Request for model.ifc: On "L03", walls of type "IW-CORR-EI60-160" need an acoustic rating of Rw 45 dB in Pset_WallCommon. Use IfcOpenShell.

First a look at what the model holds.

```python
import ifcopenshell
import ifcopenshell.util.element

model = ifcopenshell.open("model.ifc")
print(model.schema)
storey = next(s for s in model.by_type("IfcBuildingStorey") if s.Name == "L03")
walls = [e for e in ifcopenshell.util.element.get_decomposition(storey) if e.is_a("IfcWall")]
seen = {}
for e in walls:
    element_type = ifcopenshell.util.element.get_type(e)
    key = (element_type.Name if element_type != e and element_type else None, ifcopenshell.util.element.get_pset(e, "Pset_WallCommon", "AcousticRating"))
    seen[key] = seen.get(key, 0) + 1
for (name, value), count in sorted(seen.items(), key=str):
    print(count, "x", name, "|", value)
```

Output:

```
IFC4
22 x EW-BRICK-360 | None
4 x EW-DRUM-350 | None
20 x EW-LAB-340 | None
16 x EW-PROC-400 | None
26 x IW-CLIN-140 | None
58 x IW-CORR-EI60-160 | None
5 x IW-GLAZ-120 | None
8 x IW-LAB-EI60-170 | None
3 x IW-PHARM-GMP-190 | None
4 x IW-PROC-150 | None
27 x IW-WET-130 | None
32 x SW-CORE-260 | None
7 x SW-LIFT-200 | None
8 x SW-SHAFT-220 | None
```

```python
import ifcopenshell
import ifcopenshell.api.pset
import ifcopenshell.util.element

model = ifcopenshell.open("model.ifc")

storey = next(s for s in model.by_type("IfcBuildingStorey") if s.Name == "L03")
walls = [e for e in ifcopenshell.util.element.get_decomposition(storey) if e.is_a("IfcWall")]

count = 0
for e in walls:
    element_type = ifcopenshell.util.element.get_type(e)
    if element_type in (None, e) or element_type.Name != "IW-CORR-EI60-160":
        continue
    # add_pset returns the element's existing set when there is one.
    pset = ifcopenshell.api.pset.add_pset(model, product=e, name="Pset_WallCommon")
    ifcopenshell.api.pset.edit_pset(model, pset=pset, properties={"AcousticRating": "Rw 45 dB"})
    count += 1

print(count, "walls updated")

model.write("model_updated.ifc")
```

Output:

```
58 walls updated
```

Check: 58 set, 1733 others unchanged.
